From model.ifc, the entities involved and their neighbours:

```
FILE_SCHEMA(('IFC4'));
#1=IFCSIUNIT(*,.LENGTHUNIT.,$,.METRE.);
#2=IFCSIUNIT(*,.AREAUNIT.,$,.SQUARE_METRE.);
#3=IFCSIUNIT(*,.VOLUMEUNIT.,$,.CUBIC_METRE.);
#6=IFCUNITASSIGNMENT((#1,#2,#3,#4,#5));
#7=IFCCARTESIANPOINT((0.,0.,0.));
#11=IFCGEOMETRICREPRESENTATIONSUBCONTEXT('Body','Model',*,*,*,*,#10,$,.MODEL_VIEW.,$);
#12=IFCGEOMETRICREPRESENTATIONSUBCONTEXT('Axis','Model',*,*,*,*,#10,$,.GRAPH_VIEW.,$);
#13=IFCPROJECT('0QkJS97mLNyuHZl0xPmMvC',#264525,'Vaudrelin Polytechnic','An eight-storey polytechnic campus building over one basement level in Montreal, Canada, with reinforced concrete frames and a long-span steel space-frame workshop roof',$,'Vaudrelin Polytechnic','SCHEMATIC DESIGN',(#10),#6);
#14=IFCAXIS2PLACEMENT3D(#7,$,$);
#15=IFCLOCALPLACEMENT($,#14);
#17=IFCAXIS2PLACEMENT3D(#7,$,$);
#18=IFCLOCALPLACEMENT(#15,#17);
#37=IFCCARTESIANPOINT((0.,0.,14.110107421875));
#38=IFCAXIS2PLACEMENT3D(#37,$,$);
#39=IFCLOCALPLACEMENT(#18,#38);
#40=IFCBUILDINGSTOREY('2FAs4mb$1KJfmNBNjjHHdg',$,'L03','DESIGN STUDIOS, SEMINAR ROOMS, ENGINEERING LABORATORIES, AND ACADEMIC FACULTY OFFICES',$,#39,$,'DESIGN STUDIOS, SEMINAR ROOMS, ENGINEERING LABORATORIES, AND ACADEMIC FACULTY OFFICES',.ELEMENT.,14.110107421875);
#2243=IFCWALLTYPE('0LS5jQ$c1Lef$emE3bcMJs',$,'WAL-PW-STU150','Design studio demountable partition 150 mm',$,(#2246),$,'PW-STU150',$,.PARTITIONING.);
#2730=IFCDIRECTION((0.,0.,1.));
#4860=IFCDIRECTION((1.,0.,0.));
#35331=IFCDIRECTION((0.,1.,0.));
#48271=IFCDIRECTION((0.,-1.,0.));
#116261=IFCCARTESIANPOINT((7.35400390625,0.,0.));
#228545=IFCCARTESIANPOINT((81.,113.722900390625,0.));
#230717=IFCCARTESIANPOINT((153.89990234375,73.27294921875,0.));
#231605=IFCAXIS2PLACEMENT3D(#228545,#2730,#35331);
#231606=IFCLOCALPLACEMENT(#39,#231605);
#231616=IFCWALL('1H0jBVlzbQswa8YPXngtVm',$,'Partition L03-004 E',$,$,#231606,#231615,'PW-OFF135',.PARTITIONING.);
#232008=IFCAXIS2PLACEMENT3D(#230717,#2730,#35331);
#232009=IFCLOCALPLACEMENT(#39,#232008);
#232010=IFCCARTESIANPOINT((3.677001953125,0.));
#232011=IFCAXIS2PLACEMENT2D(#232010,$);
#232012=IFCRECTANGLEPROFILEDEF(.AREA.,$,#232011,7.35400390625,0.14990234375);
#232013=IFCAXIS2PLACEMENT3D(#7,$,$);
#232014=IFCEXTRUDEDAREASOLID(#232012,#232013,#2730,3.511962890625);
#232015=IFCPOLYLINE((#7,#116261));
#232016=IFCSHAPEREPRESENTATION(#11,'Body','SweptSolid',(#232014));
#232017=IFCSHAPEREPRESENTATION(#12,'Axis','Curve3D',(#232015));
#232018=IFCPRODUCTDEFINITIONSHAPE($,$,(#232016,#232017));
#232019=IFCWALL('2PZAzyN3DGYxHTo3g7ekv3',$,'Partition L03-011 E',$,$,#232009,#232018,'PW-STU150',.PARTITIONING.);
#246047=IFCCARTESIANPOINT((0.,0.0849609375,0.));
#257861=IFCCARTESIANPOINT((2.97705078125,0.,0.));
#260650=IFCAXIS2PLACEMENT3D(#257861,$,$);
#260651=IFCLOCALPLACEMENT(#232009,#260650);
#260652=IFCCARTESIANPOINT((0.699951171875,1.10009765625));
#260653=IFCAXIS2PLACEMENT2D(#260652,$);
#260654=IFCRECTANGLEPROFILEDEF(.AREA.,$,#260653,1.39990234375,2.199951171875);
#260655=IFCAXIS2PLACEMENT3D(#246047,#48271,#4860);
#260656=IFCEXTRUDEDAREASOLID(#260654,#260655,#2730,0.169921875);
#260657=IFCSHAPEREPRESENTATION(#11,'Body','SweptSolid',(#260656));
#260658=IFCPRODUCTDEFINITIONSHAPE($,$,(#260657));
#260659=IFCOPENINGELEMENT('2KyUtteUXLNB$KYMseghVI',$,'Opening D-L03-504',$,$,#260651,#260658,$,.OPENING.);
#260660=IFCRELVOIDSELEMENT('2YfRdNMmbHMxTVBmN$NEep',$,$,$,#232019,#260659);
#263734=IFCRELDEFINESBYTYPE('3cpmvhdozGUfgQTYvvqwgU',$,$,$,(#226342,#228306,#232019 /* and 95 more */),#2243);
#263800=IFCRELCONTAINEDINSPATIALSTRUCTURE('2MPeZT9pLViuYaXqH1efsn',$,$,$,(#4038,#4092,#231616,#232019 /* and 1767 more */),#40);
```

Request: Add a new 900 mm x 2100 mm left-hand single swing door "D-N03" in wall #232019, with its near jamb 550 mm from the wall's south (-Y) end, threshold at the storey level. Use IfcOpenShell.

```python
import numpy as np
import ifcopenshell
import ifcopenshell.api.feature
import ifcopenshell.api.geometry
import ifcopenshell.api.root
import ifcopenshell.api.spatial
import ifcopenshell.geom
import ifcopenshell.util.element
import ifcopenshell.util.placement
import ifcopenshell.util.representation
import ifcopenshell.util.shape
import ifcopenshell.util.unit

model = ifcopenshell.open("model.ifc")
unit_scale = ifcopenshell.util.unit.calculate_unit_scale(model)
settings = ifcopenshell.geom.settings()


def volume(element):
    """Net volume in cubic metres, openings subtracted."""
    shape = ifcopenshell.geom.create_shape(settings, element)
    return ifcopenshell.util.shape.get_volume(shape.geometry)


wall = model.by_id(232019)
storey = ifcopenshell.util.element.get_container(wall, ifc_class="IfcBuildingStorey")
context = ifcopenshell.util.representation.get_context(model, "Model", "Body", "MODEL_VIEW")
before = volume(wall)

width, height, from_end, sill = 0.9, 2.1, 0.55, 0.0  # metres

# The wall runs along its own X axis, and the end named is its -X end.
wall_shape = ifcopenshell.geom.create_shape(settings, wall)
x, y, z = ifcopenshell.util.shape.get_vertices(wall_shape.geometry).T
start = x.min() + from_end
face, thickness = float(y.min()), float(y.max() - y.min())
wall_matrix = ifcopenshell.util.placement.get_local_placement(wall.ObjectPlacement)
level = ifcopenshell.util.placement.get_local_placement(storey.ObjectPlacement)[2, 3]


def in_wall(x, y):
    """Placement at x, y metres in the wall's axes, at sill height."""
    matrix = wall_matrix.copy()
    matrix[:, 3] = wall_matrix @ np.array([x / unit_scale, y / unit_scale, 0.0, 1.0])
    matrix[2, 3] = level + sill / unit_scale
    return matrix


# Opening: a box that overshoots both wall faces by 50 mm.
opening = ifcopenshell.api.root.create_entity(model, ifc_class="IfcOpeningElement", predefined_type="OPENING")
box = ifcopenshell.api.geometry.add_wall_representation(
    model, context=context, length=width, height=height, thickness=thickness + 0.1
)
ifcopenshell.api.geometry.assign_representation(model, product=opening, representation=box)
ifcopenshell.api.geometry.edit_object_placement(model, product=opening, matrix=in_wall(start, face - 0.05), is_si=False)
ifcopenshell.api.feature.add_feature(model, feature=opening, element=wall)

door = ifcopenshell.api.root.create_entity(model, ifc_class="IfcDoor", name="D-N03", predefined_type="DOOR")
door.OverallWidth, door.OverallHeight = width / unit_scale, height / unit_scale
door.OperationType = "SINGLE_SWING_LEFT"
body = ifcopenshell.api.geometry.add_door_representation(
    model,
    context=context,
    overall_width=door.OverallWidth,
    overall_height=door.OverallHeight,
    operation_type="SINGLE_SWING_LEFT",
    lining_properties={"LiningDepth": thickness / unit_scale, "ThresholdDepth": thickness / unit_scale},
)
ifcopenshell.api.geometry.assign_representation(model, product=door, representation=body)
ifcopenshell.api.spatial.assign_container(model, products=[door], relating_structure=storey)
ifcopenshell.api.feature.add_filling(model, opening=opening, element=door)

# The lining spans the wall, so the door starts at the wall face.
ifcopenshell.api.geometry.edit_object_placement(model, product=door, matrix=in_wall(start, face), is_si=False)

after = volume(wall)

print(f"wall volume {before:.3f} -> {after:.3f} m3")

model.write("model_updated.ifc")
```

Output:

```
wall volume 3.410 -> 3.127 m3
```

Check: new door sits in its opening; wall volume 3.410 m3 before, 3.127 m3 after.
